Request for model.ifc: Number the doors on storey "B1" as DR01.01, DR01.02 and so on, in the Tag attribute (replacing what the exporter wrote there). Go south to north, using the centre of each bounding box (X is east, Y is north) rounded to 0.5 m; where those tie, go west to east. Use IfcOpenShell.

First a look at what the model holds.

```python
import ifcopenshell
import ifcopenshell.util.element
import ifcopenshell.util.placement

model = ifcopenshell.open("model.ifc")
print(model.schema)
storey = next(s for s in model.by_type("IfcBuildingStorey") if s.Name == "B1")
doors = [e for e in ifcopenshell.util.element.get_decomposition(storey) if e.is_a("IfcDoor")]
for e in sorted(doors, key=lambda e: e.id()):
    origin = ifcopenshell.util.placement.get_local_placement(e.ObjectPlacement)[:3, 3]
    print(e.id(), e.Tag, e.Name, origin.round(2) + 0.0, sep=" | ")
```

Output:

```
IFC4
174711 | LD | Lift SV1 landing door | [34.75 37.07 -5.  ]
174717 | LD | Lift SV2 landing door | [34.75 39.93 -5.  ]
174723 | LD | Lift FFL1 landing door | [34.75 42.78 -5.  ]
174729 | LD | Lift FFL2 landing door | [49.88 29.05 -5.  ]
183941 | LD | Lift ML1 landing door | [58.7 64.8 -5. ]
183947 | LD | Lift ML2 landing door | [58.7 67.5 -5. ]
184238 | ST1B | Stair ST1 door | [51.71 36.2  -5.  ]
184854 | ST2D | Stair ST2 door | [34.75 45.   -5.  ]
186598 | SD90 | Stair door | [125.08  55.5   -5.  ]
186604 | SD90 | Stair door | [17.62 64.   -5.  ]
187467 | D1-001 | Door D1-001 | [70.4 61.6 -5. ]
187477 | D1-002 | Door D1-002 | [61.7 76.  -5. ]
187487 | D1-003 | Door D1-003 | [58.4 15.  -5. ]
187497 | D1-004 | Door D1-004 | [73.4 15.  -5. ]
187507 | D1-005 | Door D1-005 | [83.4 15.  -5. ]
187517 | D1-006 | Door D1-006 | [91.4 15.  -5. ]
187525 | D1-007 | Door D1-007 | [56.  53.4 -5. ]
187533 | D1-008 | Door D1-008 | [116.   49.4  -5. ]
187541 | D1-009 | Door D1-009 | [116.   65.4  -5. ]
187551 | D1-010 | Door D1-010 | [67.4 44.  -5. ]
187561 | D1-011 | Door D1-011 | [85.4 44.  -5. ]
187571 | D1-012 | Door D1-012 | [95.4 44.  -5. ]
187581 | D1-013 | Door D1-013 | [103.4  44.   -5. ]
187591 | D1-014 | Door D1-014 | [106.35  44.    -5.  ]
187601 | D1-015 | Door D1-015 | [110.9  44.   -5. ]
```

```python
import ifcopenshell
import ifcopenshell.geom
import ifcopenshell.util.element
import ifcopenshell.util.shape

model = ifcopenshell.open("model.ifc")
settings = ifcopenshell.geom.settings()
settings.set("use-world-coords", True)


def centre(element):
    shape = ifcopenshell.geom.create_shape(settings, element)
    return ifcopenshell.util.shape.get_bbox_centroid(shape.geometry)


storey = next(s for s in model.by_type("IfcBuildingStorey") if s.Name == "B1")
doors = [e for e in ifcopenshell.util.element.get_decomposition(storey) if e.is_a("IfcDoor")]

# Insertion points can sit at a corner or the storey origin, so sort by the geometry (in metres).
centres = {e: centre(e) for e in doors}
doors.sort(key=lambda e: (round(centres[e][1] / 0.5), centres[e][0]))

for i, e in enumerate(doors, start=1):
    number = f"DR01.{i:02d}"
    e.Tag = number
    print(e.id(), number)

model.write("model_updated.ifc")
```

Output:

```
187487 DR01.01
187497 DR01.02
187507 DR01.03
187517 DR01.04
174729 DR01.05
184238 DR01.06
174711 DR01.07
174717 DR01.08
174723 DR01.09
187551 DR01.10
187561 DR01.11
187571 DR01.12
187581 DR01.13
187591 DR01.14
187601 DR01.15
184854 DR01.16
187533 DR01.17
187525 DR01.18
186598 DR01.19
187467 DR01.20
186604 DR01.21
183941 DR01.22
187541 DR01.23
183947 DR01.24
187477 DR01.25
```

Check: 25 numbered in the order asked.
